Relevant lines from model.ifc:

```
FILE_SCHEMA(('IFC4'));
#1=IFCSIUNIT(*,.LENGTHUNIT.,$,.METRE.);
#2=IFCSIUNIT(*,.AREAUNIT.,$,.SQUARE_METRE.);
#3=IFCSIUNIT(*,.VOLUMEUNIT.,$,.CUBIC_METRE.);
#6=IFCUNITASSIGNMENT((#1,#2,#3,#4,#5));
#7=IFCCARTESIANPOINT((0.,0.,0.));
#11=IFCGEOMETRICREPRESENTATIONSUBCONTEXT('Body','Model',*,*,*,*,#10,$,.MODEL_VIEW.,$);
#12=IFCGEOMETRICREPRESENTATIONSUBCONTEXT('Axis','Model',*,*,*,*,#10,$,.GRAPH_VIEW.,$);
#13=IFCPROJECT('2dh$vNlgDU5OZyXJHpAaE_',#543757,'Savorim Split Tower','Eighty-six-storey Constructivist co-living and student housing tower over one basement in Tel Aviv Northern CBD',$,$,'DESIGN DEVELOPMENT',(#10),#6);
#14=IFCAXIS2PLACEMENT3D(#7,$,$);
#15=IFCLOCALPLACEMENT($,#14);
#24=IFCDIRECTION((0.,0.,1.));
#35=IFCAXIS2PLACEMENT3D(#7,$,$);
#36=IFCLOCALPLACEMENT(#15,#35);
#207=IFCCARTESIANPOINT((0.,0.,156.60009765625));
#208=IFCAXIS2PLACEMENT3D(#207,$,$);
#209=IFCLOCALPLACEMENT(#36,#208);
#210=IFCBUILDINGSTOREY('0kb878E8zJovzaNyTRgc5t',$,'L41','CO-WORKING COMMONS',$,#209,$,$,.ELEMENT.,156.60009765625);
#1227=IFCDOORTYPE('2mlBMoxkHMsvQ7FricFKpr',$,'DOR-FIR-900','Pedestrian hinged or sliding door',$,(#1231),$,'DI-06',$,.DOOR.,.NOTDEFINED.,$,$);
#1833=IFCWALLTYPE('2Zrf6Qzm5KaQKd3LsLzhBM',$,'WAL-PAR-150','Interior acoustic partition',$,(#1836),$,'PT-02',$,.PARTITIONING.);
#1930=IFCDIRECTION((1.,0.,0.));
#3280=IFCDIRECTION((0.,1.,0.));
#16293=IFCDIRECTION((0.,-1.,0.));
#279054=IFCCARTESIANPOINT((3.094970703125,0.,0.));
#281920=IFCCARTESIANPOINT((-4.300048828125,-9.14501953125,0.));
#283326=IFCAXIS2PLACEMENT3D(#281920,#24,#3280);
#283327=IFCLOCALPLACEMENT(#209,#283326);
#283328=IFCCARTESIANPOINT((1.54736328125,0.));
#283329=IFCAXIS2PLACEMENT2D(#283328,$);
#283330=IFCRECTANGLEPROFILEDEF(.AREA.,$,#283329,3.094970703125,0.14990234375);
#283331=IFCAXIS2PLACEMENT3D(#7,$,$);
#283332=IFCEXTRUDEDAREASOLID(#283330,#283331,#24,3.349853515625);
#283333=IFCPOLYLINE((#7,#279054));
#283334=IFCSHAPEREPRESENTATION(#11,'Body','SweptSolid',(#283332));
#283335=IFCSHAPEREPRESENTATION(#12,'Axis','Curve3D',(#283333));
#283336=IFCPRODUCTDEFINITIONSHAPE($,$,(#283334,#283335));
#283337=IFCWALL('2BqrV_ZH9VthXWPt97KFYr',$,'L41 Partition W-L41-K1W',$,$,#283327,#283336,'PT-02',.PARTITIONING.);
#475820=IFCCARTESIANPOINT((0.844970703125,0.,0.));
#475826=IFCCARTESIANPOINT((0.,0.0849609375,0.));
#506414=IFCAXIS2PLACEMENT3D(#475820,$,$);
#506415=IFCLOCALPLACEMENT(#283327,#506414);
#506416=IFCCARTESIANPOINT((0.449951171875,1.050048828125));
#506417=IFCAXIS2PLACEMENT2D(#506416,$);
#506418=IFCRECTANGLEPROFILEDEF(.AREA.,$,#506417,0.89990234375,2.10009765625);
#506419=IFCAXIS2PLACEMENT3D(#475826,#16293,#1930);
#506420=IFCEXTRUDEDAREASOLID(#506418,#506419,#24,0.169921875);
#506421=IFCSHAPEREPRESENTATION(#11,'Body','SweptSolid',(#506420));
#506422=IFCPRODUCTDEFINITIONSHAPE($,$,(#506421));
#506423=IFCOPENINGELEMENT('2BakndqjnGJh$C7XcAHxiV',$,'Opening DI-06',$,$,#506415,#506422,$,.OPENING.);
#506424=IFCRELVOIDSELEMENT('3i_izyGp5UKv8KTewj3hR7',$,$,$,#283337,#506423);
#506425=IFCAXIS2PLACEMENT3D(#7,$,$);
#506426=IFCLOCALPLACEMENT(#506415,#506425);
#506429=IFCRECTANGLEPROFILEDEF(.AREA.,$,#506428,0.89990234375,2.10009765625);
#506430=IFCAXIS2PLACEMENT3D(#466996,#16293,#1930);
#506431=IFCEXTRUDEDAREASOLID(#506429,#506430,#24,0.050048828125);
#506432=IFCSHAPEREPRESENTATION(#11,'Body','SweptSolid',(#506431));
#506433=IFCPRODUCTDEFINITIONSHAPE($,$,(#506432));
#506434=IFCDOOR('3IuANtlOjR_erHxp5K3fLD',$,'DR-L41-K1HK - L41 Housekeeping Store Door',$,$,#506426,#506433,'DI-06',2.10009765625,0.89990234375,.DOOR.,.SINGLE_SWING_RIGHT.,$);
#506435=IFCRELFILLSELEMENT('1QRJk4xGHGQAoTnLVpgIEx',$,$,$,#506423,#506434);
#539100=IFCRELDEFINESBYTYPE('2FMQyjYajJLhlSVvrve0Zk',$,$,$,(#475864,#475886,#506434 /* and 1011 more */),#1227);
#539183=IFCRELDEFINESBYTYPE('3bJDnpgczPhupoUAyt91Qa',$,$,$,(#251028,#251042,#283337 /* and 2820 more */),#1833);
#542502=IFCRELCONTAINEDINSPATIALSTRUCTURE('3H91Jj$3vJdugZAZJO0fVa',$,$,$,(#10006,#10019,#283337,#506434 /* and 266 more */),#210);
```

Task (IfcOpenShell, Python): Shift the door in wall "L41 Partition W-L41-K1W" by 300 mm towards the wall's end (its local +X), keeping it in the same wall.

```python
import ifcopenshell
import ifcopenshell.api.geometry
import ifcopenshell.util.placement
import ifcopenshell.util.unit

model = ifcopenshell.open("model.ifc")
unit_scale = ifcopenshell.util.unit.calculate_unit_scale(model)

door = model.by_id(506434)
opening = door.FillsVoids[0].RelatingOpeningElement
wall = opening.VoidsElements[0].RelatingBuildingElement

wall_matrix = ifcopenshell.util.placement.get_local_placement(wall.ObjectPlacement)
shift = wall_matrix[:3, 0] * 0.3 / unit_scale
before = ifcopenshell.util.placement.get_local_placement(door.ObjectPlacement)[:3, 3].copy()

# The door is placed relative to its opening, so it follows when the opening moves.
matrix = ifcopenshell.util.placement.get_local_placement(opening.ObjectPlacement)
matrix[:3, 3] += shift
ifcopenshell.api.geometry.edit_object_placement(
    model, product=opening, matrix=matrix, is_si=False, should_transform_children=True
)

after = ifcopenshell.util.placement.get_local_placement(door.ObjectPlacement)[:3, 3]
print("door moved by", (after - before).round(3) + 0.0)

model.write("model_updated.ifc")
```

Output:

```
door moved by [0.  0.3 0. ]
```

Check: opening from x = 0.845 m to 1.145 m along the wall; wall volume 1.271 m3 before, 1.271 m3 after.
